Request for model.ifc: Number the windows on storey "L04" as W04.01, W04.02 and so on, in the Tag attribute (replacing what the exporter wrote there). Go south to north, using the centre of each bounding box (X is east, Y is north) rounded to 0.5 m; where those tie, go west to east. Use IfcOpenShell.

First a look at what the model holds.

```python
import ifcopenshell
import ifcopenshell.util.element
import ifcopenshell.util.placement

model = ifcopenshell.open("model.ifc")
print(model.schema)
storey = next(s for s in model.by_type("IfcBuildingStorey") if s.Name == "L04")
windows = [e for e in ifcopenshell.util.element.get_decomposition(storey) if e.is_a("IfcWindow")]
for e in sorted(windows, key=lambda e: e.id()):
    origin = ifcopenshell.util.placement.get_local_placement(e.ObjectPlacement)[:3, 3]
    print(e.id(), e.Tag, e.Name, origin.round(2) + 0.0, sep=" | ")
```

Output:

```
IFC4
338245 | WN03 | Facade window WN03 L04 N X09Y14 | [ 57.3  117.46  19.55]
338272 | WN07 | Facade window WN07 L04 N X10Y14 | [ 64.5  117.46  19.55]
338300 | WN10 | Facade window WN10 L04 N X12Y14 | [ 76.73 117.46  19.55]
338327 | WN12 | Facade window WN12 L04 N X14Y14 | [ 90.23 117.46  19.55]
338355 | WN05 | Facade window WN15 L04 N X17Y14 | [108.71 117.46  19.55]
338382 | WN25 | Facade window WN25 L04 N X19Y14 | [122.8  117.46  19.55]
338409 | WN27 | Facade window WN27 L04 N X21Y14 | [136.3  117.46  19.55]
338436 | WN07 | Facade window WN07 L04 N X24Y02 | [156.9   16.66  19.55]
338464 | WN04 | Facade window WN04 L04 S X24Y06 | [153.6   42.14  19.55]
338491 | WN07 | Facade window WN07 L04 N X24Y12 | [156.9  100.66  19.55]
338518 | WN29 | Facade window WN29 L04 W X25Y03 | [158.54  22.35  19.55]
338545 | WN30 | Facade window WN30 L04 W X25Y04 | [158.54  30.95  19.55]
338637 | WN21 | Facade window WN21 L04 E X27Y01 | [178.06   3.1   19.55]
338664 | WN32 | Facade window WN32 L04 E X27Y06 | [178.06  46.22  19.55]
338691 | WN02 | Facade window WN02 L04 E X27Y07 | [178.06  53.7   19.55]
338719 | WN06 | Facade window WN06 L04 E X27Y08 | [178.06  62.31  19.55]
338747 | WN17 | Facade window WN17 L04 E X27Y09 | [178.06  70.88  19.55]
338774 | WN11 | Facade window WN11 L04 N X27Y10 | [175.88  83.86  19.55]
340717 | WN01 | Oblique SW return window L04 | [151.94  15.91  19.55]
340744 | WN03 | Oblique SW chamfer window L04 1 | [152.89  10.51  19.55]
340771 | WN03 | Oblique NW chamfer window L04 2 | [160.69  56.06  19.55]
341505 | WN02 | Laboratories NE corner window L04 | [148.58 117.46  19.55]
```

```python
import ifcopenshell
import ifcopenshell.geom
import ifcopenshell.util.element
import ifcopenshell.util.shape

model = ifcopenshell.open("model.ifc")
settings = ifcopenshell.geom.settings()
settings.set("use-world-coords", True)


def centre(element):
    shape = ifcopenshell.geom.create_shape(settings, element)
    return ifcopenshell.util.shape.get_bbox_centroid(shape.geometry)


storey = next(s for s in model.by_type("IfcBuildingStorey") if s.Name == "L04")
windows = [e for e in ifcopenshell.util.element.get_decomposition(storey) if e.is_a("IfcWindow")]

# Insertion points can sit at a corner or the storey origin, so sort by the geometry (in metres).
centres = {e: centre(e) for e in windows}
windows.sort(key=lambda e: (round(centres[e][1] / 0.5), centres[e][0]))

for i, e in enumerate(windows, start=1):
    number = f"W04.{i:02d}"
    e.Tag = number
    print(e.id(), number)

model.write("model_edited.ifc")
```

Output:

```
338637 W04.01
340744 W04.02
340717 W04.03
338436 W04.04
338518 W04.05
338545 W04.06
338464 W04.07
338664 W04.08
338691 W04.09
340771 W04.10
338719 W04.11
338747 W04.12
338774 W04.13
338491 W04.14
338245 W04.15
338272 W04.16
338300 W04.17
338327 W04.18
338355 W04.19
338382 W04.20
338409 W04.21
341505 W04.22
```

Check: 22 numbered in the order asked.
